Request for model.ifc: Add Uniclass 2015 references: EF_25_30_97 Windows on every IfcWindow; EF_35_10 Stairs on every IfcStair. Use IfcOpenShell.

First a look at what the model holds.

```python
import ifcopenshell

model = ifcopenshell.open("model.ifc")
print(model.schema)
print("classifications:", [c.Name for c in model.by_type("IfcClassification")])
for ifc_class in ("IfcDoor", "IfcRoof", "IfcStair", "IfcWall", "IfcWindow"):
    print(ifc_class, len(model.by_type(ifc_class)))
```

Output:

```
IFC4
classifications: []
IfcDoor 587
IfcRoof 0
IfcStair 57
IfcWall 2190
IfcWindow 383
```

```python
import ifcopenshell
import ifcopenshell.api.classification

model = ifcopenshell.open("model.ifc")

system = ifcopenshell.api.classification.add_classification(model, classification="Uniclass 2015")

codes = {
    "IfcWindow": ("EF_25_30_97", "Windows"),
    "IfcStair": ("EF_35_10", "Stairs"),
}
for ifc_class, (code, name) in codes.items():
    products = model.by_type(ifc_class)
    ifcopenshell.api.classification.add_reference(
        model, products=products, classification=system, identification=code, name=name
    )
    print(code, len(products))

model.write("model_rev.ifc")
```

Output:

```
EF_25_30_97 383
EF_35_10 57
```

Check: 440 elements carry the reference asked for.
